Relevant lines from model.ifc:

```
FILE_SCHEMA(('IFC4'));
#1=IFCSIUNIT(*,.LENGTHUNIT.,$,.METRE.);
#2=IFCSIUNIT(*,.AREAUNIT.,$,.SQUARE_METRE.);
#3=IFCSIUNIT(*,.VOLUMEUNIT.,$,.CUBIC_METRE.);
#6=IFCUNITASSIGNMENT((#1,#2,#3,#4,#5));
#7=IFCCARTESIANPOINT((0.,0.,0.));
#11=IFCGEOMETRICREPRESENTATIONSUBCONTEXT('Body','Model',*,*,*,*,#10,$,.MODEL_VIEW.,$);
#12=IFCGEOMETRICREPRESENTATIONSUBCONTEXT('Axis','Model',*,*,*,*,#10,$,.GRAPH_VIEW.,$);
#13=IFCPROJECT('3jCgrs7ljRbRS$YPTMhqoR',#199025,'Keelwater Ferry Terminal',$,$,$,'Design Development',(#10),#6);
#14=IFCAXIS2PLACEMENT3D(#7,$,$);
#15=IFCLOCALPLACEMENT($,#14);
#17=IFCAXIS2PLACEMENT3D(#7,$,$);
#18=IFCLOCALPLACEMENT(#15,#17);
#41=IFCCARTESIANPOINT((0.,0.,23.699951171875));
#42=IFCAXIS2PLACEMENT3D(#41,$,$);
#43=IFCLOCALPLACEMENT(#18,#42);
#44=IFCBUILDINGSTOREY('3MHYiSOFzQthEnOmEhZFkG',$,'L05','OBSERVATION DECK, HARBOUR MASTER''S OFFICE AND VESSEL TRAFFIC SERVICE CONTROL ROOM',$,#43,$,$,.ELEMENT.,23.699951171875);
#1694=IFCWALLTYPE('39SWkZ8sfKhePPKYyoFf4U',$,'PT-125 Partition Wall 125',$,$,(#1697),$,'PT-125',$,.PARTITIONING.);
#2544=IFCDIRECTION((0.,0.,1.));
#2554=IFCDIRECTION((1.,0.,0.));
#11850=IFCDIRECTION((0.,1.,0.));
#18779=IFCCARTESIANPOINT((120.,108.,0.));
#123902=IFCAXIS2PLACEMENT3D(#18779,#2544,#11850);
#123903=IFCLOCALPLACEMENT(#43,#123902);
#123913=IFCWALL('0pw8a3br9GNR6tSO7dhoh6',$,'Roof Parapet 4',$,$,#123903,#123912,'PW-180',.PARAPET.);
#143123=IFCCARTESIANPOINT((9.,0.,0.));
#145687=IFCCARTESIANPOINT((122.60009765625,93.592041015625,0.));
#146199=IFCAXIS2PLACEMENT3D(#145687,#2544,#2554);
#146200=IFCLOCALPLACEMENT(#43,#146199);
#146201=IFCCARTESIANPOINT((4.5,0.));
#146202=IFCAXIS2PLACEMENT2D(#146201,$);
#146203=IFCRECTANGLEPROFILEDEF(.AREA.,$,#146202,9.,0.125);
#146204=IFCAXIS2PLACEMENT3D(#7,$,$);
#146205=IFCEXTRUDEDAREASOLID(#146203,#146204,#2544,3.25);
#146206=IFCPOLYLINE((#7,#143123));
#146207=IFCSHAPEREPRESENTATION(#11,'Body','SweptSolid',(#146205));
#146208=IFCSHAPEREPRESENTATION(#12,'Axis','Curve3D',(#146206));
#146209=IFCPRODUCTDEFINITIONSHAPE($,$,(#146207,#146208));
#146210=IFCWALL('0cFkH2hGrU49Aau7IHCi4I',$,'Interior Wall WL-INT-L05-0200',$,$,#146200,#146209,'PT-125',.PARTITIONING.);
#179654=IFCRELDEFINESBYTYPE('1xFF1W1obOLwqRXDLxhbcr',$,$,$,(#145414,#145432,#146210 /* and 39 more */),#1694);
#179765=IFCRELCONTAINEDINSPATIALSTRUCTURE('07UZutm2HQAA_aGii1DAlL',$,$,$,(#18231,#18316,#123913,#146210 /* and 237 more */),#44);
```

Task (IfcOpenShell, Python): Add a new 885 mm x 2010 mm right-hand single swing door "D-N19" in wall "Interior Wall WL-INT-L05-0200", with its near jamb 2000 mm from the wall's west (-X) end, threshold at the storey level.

```python
import numpy as np
import ifcopenshell
import ifcopenshell.api.feature
import ifcopenshell.api.geometry
import ifcopenshell.api.root
import ifcopenshell.api.spatial
import ifcopenshell.geom
import ifcopenshell.util.element
import ifcopenshell.util.placement
import ifcopenshell.util.representation
import ifcopenshell.util.shape
import ifcopenshell.util.unit

model = ifcopenshell.open("model.ifc")
unit_scale = ifcopenshell.util.unit.calculate_unit_scale(model)
settings = ifcopenshell.geom.settings()


def volume(element):
    """Net volume in cubic metres, openings subtracted."""
    shape = ifcopenshell.geom.create_shape(settings, element)
    return ifcopenshell.util.shape.get_volume(shape.geometry)


wall = model.by_guid("0cFkH2hGrU49Aau7IHCi4I")
storey = ifcopenshell.util.element.get_container(wall, ifc_class="IfcBuildingStorey")
context = ifcopenshell.util.representation.get_context(model, "Model", "Body", "MODEL_VIEW")
before = volume(wall)

width, height, from_end, sill = 0.885, 2.01, 2, 0.0  # metres

# The wall runs along its own X axis, and the end named is its -X end.
wall_shape = ifcopenshell.geom.create_shape(settings, wall)
x, y, z = ifcopenshell.util.shape.get_vertices(wall_shape.geometry).T
start = x.min() + from_end
face, thickness = float(y.min()), float(y.max() - y.min())
wall_matrix = ifcopenshell.util.placement.get_local_placement(wall.ObjectPlacement)
level = ifcopenshell.util.placement.get_local_placement(storey.ObjectPlacement)[2, 3]


def in_wall(x, y):
    """Placement at x, y metres in the wall's axes, at sill height."""
    matrix = wall_matrix.copy()
    matrix[:, 3] = wall_matrix @ np.array([x / unit_scale, y / unit_scale, 0.0, 1.0])
    matrix[2, 3] = level + sill / unit_scale
    return matrix


# Opening: a box that overshoots both wall faces by 50 mm.
opening = ifcopenshell.api.root.create_entity(model, ifc_class="IfcOpeningElement", predefined_type="OPENING")
box = ifcopenshell.api.geometry.add_wall_representation(
    model, context=context, length=width, height=height, thickness=thickness + 0.1
)
ifcopenshell.api.geometry.assign_representation(model, product=opening, representation=box)
ifcopenshell.api.geometry.edit_object_placement(model, product=opening, matrix=in_wall(start, face - 0.05), is_si=False)
ifcopenshell.api.feature.add_feature(model, feature=opening, element=wall)

door = ifcopenshell.api.root.create_entity(model, ifc_class="IfcDoor", name="D-N19", predefined_type="DOOR")
door.OverallWidth, door.OverallHeight = width / unit_scale, height / unit_scale
door.OperationType = "SINGLE_SWING_RIGHT"
body = ifcopenshell.api.geometry.add_door_representation(
    model,
    context=context,
    overall_width=door.OverallWidth,
    overall_height=door.OverallHeight,
    operation_type="SINGLE_SWING_RIGHT",
    lining_properties={"LiningDepth": thickness / unit_scale, "ThresholdDepth": thickness / unit_scale},
)
ifcopenshell.api.geometry.assign_representation(model, product=door, representation=body)
ifcopenshell.api.spatial.assign_container(model, products=[door], relating_structure=storey)
ifcopenshell.api.feature.add_filling(model, opening=opening, element=door)

# The lining spans the wall, so the door starts at the wall face.
ifcopenshell.api.geometry.edit_object_placement(model, product=door, matrix=in_wall(start, face), is_si=False)

after = volume(wall)

print(f"wall volume {before:.3f} -> {after:.3f} m3")

model.write("model_updated.ifc")
```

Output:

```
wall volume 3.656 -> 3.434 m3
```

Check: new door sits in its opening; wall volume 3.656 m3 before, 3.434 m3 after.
